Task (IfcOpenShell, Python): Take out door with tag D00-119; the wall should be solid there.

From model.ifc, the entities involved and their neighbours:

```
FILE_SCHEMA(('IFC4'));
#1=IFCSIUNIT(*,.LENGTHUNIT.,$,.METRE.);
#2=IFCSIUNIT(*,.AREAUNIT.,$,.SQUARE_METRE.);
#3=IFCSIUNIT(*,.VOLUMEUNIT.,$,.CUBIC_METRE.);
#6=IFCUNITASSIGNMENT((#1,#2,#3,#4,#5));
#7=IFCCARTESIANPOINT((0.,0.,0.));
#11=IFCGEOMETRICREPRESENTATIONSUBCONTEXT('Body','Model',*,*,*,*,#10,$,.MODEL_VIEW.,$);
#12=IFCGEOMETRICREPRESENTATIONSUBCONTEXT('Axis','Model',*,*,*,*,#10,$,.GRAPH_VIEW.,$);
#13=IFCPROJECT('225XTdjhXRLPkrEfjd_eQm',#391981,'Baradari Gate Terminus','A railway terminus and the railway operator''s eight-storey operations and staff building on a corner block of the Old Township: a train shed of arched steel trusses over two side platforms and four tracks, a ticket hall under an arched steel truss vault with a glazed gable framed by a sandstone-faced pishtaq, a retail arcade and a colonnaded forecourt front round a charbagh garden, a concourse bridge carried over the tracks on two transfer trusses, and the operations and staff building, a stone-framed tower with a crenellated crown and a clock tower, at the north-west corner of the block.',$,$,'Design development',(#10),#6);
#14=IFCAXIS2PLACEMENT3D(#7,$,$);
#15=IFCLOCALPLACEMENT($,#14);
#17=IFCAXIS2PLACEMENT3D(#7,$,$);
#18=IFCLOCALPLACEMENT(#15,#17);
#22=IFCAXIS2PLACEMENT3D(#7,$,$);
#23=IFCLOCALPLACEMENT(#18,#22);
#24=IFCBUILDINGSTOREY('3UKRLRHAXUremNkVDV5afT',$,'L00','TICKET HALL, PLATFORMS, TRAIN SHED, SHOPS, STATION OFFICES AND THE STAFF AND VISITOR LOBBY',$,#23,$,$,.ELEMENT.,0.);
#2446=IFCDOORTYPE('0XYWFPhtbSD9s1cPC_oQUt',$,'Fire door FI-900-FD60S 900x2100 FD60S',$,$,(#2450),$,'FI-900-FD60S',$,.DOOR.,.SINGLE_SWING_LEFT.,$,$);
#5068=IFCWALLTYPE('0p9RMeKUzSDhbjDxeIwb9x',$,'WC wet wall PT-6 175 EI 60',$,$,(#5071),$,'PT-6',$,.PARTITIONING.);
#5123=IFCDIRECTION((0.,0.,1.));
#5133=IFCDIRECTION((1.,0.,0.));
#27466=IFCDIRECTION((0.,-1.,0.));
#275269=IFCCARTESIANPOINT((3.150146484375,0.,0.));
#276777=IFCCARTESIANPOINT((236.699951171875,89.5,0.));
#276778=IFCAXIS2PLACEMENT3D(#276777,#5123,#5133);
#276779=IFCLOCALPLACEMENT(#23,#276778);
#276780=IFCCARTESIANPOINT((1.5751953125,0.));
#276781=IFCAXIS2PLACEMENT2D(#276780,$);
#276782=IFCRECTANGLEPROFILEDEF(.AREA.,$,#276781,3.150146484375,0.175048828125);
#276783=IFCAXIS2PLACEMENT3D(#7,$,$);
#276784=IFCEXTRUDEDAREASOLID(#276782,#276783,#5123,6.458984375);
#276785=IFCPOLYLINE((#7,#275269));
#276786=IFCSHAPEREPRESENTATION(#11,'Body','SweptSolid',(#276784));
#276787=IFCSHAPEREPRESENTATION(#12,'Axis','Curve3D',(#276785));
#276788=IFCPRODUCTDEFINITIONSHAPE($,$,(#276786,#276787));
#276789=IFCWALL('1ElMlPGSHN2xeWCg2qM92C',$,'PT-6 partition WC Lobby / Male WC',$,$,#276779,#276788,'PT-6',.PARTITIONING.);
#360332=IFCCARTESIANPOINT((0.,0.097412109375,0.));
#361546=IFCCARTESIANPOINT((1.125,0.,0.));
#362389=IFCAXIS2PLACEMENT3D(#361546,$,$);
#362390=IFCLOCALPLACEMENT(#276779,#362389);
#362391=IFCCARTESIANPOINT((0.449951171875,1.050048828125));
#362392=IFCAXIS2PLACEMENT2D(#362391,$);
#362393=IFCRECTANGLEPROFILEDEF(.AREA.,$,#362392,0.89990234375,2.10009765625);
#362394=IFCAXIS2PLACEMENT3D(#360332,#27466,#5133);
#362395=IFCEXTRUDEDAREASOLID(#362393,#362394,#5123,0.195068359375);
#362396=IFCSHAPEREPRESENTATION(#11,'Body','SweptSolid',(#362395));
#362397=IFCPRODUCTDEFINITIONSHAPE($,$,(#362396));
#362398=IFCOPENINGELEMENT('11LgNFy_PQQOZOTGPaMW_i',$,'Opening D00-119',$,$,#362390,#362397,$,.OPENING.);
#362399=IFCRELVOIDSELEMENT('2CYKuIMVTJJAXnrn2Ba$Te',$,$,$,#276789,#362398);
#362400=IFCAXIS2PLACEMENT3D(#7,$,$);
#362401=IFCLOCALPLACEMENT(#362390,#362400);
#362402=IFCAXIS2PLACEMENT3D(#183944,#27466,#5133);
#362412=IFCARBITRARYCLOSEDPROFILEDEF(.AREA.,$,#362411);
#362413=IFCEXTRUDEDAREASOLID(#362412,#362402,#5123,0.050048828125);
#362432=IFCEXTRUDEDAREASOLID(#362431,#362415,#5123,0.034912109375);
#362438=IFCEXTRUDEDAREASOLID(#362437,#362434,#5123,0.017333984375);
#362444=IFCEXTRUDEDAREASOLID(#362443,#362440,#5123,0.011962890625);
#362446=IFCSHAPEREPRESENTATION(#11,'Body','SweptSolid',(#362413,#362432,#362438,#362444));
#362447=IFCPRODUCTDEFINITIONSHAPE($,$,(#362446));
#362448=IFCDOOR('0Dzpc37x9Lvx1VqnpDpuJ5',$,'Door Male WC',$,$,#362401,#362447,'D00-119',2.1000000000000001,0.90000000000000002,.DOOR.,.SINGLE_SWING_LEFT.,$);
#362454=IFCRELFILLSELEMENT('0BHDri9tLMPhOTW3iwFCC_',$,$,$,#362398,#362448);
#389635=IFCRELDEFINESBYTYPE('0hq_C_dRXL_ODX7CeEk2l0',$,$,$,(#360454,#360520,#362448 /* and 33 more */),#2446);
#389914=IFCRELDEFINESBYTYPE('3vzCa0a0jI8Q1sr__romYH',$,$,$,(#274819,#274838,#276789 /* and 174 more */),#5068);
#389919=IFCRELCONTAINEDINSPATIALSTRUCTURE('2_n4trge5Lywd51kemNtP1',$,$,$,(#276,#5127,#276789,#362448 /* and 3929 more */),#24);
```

```python
import ifcopenshell
import ifcopenshell.api.feature
import ifcopenshell.api.root
import ifcopenshell.geom
import ifcopenshell.util.shape

model = ifcopenshell.open("model.ifc")
settings = ifcopenshell.geom.settings()


def volume(element):
    """Net volume in cubic metres, openings subtracted."""
    shape = ifcopenshell.geom.create_shape(settings, element)
    return ifcopenshell.util.shape.get_volume(shape.geometry)


door = model.by_guid("0Dzpc37x9Lvx1VqnpDpuJ5")
opening = door.FillsVoids[0].RelatingOpeningElement
wall = opening.VoidsElements[0].RelatingBuildingElement
before = volume(wall)

ifcopenshell.api.root.remove_product(model, product=door)
ifcopenshell.api.feature.remove_feature(model, feature=opening)

after = volume(wall)

print(f"wall volume {before:.3f} -> {after:.3f} m3")

model.write("model_updated.ifc")
```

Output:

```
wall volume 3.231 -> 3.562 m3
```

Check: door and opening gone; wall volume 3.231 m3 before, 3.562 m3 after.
